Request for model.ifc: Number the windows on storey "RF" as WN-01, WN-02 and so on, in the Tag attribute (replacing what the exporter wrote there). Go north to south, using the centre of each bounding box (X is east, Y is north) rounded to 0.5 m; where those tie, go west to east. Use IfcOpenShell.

First a look at what the model holds.

```python
import ifcopenshell
import ifcopenshell.util.element
import ifcopenshell.util.placement

model = ifcopenshell.open("model.ifc")
print(model.schema)
storey = next(s for s in model.by_type("IfcBuildingStorey") if s.Name == "RF")
windows = [e for e in ifcopenshell.util.element.get_decomposition(storey) if e.is_a("IfcWindow")]
for e in sorted(windows, key=lambda e: e.id()):
    origin = ifcopenshell.util.placement.get_local_placement(e.ObjectPlacement)[:3, 3]
    print(e.id(), e.Tag, e.Name, origin.round(2) + 0.0, sep=" | ")
```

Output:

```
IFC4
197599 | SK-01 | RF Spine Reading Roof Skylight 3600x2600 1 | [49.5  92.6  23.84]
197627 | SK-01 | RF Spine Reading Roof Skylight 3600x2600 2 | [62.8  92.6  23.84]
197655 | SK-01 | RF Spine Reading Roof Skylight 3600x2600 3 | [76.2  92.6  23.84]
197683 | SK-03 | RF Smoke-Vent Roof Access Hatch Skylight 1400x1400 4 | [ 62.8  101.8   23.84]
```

```python
import ifcopenshell
import ifcopenshell.geom
import ifcopenshell.util.element
import ifcopenshell.util.shape

model = ifcopenshell.open("model.ifc")
settings = ifcopenshell.geom.settings()
settings.set("use-world-coords", True)


def centre(element):
    shape = ifcopenshell.geom.create_shape(settings, element)
    return ifcopenshell.util.shape.get_bbox_centroid(shape.geometry)


storey = next(s for s in model.by_type("IfcBuildingStorey") if s.Name == "RF")
windows = [e for e in ifcopenshell.util.element.get_decomposition(storey) if e.is_a("IfcWindow")]

# Insertion points can sit at a corner or the storey origin, so sort by the geometry (in metres).
centres = {e: centre(e) for e in windows}
windows.sort(key=lambda e: (-round(centres[e][1] / 0.5), centres[e][0]))

for i, e in enumerate(windows, start=1):
    number = f"WN-{i:02d}"
    e.Tag = number
    print(e.id(), number)

model.write("model_rev.ifc")
```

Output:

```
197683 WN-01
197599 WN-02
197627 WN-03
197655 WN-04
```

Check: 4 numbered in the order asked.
